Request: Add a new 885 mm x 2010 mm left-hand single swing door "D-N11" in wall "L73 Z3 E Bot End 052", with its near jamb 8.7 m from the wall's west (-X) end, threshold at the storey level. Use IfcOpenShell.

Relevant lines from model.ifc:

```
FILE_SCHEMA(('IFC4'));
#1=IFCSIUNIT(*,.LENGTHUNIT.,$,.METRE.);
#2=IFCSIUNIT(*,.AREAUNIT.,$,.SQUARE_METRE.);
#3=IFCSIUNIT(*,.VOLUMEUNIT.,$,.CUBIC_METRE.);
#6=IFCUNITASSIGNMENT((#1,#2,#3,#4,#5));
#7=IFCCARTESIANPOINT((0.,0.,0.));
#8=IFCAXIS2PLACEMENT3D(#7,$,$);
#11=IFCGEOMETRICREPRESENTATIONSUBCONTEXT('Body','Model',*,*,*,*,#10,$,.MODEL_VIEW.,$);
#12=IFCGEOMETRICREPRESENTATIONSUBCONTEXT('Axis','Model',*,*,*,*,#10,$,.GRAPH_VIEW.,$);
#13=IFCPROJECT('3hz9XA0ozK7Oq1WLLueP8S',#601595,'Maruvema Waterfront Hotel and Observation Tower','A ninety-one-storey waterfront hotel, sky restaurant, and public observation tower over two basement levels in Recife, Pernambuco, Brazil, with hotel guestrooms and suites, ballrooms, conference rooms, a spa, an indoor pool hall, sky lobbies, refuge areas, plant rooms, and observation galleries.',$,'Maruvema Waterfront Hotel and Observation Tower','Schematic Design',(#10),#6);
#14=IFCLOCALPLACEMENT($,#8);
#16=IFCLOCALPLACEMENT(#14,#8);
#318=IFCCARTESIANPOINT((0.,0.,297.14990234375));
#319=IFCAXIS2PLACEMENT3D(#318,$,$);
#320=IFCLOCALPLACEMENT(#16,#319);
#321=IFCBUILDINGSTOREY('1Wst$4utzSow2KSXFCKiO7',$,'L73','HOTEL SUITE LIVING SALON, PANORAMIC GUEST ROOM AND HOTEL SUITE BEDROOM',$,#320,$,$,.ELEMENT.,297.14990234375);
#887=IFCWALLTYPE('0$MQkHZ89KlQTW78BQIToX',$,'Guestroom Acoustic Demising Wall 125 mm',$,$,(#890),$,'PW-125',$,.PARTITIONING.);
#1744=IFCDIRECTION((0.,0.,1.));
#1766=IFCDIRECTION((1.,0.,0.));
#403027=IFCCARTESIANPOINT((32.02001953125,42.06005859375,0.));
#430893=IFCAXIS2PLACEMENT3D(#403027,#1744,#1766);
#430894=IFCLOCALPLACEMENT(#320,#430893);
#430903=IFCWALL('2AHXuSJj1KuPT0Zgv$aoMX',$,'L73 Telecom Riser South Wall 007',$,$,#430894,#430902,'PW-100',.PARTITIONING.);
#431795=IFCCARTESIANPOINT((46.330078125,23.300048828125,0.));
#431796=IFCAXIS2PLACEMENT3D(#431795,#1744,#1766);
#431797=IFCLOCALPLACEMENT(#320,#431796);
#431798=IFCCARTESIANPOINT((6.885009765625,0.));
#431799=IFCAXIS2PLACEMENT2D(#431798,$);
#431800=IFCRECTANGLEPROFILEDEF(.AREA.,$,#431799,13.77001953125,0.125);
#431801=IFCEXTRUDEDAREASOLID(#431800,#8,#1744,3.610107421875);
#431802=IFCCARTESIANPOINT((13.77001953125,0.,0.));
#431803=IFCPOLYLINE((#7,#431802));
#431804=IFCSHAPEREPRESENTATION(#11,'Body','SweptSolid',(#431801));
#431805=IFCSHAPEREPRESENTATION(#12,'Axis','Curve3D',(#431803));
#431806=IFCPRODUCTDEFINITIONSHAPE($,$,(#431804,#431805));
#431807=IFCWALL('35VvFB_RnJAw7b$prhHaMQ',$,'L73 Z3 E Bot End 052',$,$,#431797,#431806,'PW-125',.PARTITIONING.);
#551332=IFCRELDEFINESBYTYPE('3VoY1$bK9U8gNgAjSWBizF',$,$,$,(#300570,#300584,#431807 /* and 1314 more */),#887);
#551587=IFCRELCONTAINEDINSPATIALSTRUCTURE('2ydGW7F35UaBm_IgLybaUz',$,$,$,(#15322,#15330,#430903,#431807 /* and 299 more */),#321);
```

```python
import numpy as np
import ifcopenshell
import ifcopenshell.api.feature
import ifcopenshell.api.geometry
import ifcopenshell.api.root
import ifcopenshell.api.spatial
import ifcopenshell.geom
import ifcopenshell.util.element
import ifcopenshell.util.placement
import ifcopenshell.util.representation
import ifcopenshell.util.shape
import ifcopenshell.util.unit

model = ifcopenshell.open("model.ifc")
unit_scale = ifcopenshell.util.unit.calculate_unit_scale(model)
settings = ifcopenshell.geom.settings()


def volume(element):
    """Net volume in cubic metres, openings subtracted."""
    shape = ifcopenshell.geom.create_shape(settings, element)
    return ifcopenshell.util.shape.get_volume(shape.geometry)


wall = model.by_guid("35VvFB_RnJAw7b$prhHaMQ")
storey = ifcopenshell.util.element.get_container(wall, ifc_class="IfcBuildingStorey")
context = ifcopenshell.util.representation.get_context(model, "Model", "Body", "MODEL_VIEW")
before = volume(wall)

width, height, from_end, sill = 0.885, 2.01, 8.7, 0.0  # metres

# The wall runs along its own X axis, and the end named is its -X end.
wall_shape = ifcopenshell.geom.create_shape(settings, wall)
x, y, z = ifcopenshell.util.shape.get_vertices(wall_shape.geometry).T
start = x.min() + from_end
face, thickness = float(y.min()), float(y.max() - y.min())
wall_matrix = ifcopenshell.util.placement.get_local_placement(wall.ObjectPlacement)
level = ifcopenshell.util.placement.get_local_placement(storey.ObjectPlacement)[2, 3]


def in_wall(x, y):
    """Placement at x, y metres in the wall's axes, at sill height."""
    matrix = wall_matrix.copy()
    matrix[:, 3] = wall_matrix @ np.array([x / unit_scale, y / unit_scale, 0.0, 1.0])
    matrix[2, 3] = level + sill / unit_scale
    return matrix


# Opening: a box that overshoots both wall faces by 50 mm.
opening = ifcopenshell.api.root.create_entity(model, ifc_class="IfcOpeningElement", predefined_type="OPENING")
box = ifcopenshell.api.geometry.add_wall_representation(
    model, context=context, length=width, height=height, thickness=thickness + 0.1
)
ifcopenshell.api.geometry.assign_representation(model, product=opening, representation=box)
ifcopenshell.api.geometry.edit_object_placement(model, product=opening, matrix=in_wall(start, face - 0.05), is_si=False)
ifcopenshell.api.feature.add_feature(model, feature=opening, element=wall)

door = ifcopenshell.api.root.create_entity(model, ifc_class="IfcDoor", name="D-N11", predefined_type="DOOR")
door.OverallWidth, door.OverallHeight = width / unit_scale, height / unit_scale
door.OperationType = "SINGLE_SWING_LEFT"
body = ifcopenshell.api.geometry.add_door_representation(
    model,
    context=context,
    overall_width=door.OverallWidth,
    overall_height=door.OverallHeight,
    operation_type="SINGLE_SWING_LEFT",
    lining_properties={"LiningDepth": thickness / unit_scale, "ThresholdDepth": thickness / unit_scale},
)
ifcopenshell.api.geometry.assign_representation(model, product=door, representation=body)
ifcopenshell.api.spatial.assign_container(model, products=[door], relating_structure=storey)
ifcopenshell.api.feature.add_filling(model, opening=opening, element=door)

# The lining spans the wall, so the door starts at the wall face.
ifcopenshell.api.geometry.edit_object_placement(model, product=door, matrix=in_wall(start, face), is_si=False)

after = volume(wall)

print(f"wall volume {before:.3f} -> {after:.3f} m3")

model.write("model_rev.ifc")
```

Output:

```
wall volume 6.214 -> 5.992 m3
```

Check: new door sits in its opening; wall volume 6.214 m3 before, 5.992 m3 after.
